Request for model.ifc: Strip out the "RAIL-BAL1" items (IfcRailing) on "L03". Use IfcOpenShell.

First a look at what the model holds.

```python
import ifcopenshell
import ifcopenshell.util.element

model = ifcopenshell.open("model.ifc")
print(model.schema)
storey = next(s for s in model.by_type("IfcBuildingStorey") if s.Name == "L03")
railings = [e for e in ifcopenshell.util.element.get_decomposition(storey) if e.is_a("IfcRailing")]
seen = {}
for e in railings:
    element_type = ifcopenshell.util.element.get_type(e)
    name = element_type.Name if element_type not in (None, e) else None
    seen[name] = seen.get(name, 0) + 1
for name, count in sorted(seen.items(), key=str):
    print(count, "x", name)
```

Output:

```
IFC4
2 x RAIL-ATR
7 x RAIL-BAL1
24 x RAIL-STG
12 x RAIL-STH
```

```python
import ifcopenshell
import ifcopenshell.api.root
import ifcopenshell.util.element

model = ifcopenshell.open("model.ifc")

storey = next(s for s in model.by_type("IfcBuildingStorey") if s.Name == "L03")
railings = [e for e in ifcopenshell.util.element.get_decomposition(storey) if e.is_a("IfcRailing")]
targets = [e for e in railings if (t := ifcopenshell.util.element.get_type(e)) not in (None, e) and t.Name == "RAIL-BAL1"]

for e in targets:
    ifcopenshell.api.root.remove_product(model, product=e)
print(len(targets), "removed")

model.write("model_rev.ifc")
```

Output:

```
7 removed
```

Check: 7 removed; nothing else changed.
